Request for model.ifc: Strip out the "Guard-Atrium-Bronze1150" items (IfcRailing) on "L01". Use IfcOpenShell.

First a look at what the model holds.

```python
import ifcopenshell
import ifcopenshell.util.element

model = ifcopenshell.open("model.ifc")
print(model.schema)
storey = next(s for s in model.by_type("IfcBuildingStorey") if s.Name == "L01")
railings = [e for e in ifcopenshell.util.element.get_decomposition(storey) if e.is_a("IfcRailing")]
seen = {}
for e in railings:
    element_type = ifcopenshell.util.element.get_type(e)
    name = element_type.Name if element_type not in (None, e) else None
    seen[name] = seen.get(name, 0) + 1
for name, count in sorted(seen.items(), key=str):
    print(count, "x", name)
```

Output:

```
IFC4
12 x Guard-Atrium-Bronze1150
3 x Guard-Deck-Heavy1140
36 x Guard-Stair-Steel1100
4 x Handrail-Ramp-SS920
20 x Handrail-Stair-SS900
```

```python
import ifcopenshell
import ifcopenshell.api.root
import ifcopenshell.util.element

model = ifcopenshell.open("model.ifc")

storey = next(s for s in model.by_type("IfcBuildingStorey") if s.Name == "L01")
railings = [e for e in ifcopenshell.util.element.get_decomposition(storey) if e.is_a("IfcRailing")]
targets = [e for e in railings if (t := ifcopenshell.util.element.get_type(e)) not in (None, e) and t.Name == "Guard-Atrium-Bronze1150"]

for e in targets:
    ifcopenshell.api.root.remove_product(model, product=e)
print(len(targets), "removed")

model.write("model_edited.ifc")
```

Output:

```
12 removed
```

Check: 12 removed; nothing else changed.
